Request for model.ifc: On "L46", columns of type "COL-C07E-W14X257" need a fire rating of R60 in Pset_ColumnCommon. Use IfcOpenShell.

First a look at what the model holds.

```python
import ifcopenshell
import ifcopenshell.util.element

model = ifcopenshell.open("model.ifc")
print(model.schema)
storey = next(s for s in model.by_type("IfcBuildingStorey") if s.Name == "L46")
columns = [e for e in ifcopenshell.util.element.get_decomposition(storey) if e.is_a("IfcColumn")]
seen = {}
for e in columns:
    element_type = ifcopenshell.util.element.get_type(e)
    key = (element_type.Name if element_type != e and element_type else None, ifcopenshell.util.element.get_pset(e, "Pset_ColumnCommon", "FireRating"))
    seen[key] = seen.get(key, 0) + 1
for (name, value), count in sorted(seen.items(), key=str):
    print(count, "x", name, "|", value)
```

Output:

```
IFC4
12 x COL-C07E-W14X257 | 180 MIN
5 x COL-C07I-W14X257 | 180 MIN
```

```python
import ifcopenshell
import ifcopenshell.api.pset
import ifcopenshell.util.element

model = ifcopenshell.open("model.ifc")

storey = next(s for s in model.by_type("IfcBuildingStorey") if s.Name == "L46")
columns = [e for e in ifcopenshell.util.element.get_decomposition(storey) if e.is_a("IfcColumn")]

count = 0
for e in columns:
    element_type = ifcopenshell.util.element.get_type(e)
    if element_type in (None, e) or element_type.Name != "COL-C07E-W14X257":
        continue
    # add_pset returns the element's existing set when there is one.
    pset = ifcopenshell.api.pset.add_pset(model, product=e, name="Pset_ColumnCommon")
    ifcopenshell.api.pset.edit_pset(model, pset=pset, properties={"FireRating": "R60"})
    count += 1

print(count, "columns updated")

model.write("model-out.ifc")
```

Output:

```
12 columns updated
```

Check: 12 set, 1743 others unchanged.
